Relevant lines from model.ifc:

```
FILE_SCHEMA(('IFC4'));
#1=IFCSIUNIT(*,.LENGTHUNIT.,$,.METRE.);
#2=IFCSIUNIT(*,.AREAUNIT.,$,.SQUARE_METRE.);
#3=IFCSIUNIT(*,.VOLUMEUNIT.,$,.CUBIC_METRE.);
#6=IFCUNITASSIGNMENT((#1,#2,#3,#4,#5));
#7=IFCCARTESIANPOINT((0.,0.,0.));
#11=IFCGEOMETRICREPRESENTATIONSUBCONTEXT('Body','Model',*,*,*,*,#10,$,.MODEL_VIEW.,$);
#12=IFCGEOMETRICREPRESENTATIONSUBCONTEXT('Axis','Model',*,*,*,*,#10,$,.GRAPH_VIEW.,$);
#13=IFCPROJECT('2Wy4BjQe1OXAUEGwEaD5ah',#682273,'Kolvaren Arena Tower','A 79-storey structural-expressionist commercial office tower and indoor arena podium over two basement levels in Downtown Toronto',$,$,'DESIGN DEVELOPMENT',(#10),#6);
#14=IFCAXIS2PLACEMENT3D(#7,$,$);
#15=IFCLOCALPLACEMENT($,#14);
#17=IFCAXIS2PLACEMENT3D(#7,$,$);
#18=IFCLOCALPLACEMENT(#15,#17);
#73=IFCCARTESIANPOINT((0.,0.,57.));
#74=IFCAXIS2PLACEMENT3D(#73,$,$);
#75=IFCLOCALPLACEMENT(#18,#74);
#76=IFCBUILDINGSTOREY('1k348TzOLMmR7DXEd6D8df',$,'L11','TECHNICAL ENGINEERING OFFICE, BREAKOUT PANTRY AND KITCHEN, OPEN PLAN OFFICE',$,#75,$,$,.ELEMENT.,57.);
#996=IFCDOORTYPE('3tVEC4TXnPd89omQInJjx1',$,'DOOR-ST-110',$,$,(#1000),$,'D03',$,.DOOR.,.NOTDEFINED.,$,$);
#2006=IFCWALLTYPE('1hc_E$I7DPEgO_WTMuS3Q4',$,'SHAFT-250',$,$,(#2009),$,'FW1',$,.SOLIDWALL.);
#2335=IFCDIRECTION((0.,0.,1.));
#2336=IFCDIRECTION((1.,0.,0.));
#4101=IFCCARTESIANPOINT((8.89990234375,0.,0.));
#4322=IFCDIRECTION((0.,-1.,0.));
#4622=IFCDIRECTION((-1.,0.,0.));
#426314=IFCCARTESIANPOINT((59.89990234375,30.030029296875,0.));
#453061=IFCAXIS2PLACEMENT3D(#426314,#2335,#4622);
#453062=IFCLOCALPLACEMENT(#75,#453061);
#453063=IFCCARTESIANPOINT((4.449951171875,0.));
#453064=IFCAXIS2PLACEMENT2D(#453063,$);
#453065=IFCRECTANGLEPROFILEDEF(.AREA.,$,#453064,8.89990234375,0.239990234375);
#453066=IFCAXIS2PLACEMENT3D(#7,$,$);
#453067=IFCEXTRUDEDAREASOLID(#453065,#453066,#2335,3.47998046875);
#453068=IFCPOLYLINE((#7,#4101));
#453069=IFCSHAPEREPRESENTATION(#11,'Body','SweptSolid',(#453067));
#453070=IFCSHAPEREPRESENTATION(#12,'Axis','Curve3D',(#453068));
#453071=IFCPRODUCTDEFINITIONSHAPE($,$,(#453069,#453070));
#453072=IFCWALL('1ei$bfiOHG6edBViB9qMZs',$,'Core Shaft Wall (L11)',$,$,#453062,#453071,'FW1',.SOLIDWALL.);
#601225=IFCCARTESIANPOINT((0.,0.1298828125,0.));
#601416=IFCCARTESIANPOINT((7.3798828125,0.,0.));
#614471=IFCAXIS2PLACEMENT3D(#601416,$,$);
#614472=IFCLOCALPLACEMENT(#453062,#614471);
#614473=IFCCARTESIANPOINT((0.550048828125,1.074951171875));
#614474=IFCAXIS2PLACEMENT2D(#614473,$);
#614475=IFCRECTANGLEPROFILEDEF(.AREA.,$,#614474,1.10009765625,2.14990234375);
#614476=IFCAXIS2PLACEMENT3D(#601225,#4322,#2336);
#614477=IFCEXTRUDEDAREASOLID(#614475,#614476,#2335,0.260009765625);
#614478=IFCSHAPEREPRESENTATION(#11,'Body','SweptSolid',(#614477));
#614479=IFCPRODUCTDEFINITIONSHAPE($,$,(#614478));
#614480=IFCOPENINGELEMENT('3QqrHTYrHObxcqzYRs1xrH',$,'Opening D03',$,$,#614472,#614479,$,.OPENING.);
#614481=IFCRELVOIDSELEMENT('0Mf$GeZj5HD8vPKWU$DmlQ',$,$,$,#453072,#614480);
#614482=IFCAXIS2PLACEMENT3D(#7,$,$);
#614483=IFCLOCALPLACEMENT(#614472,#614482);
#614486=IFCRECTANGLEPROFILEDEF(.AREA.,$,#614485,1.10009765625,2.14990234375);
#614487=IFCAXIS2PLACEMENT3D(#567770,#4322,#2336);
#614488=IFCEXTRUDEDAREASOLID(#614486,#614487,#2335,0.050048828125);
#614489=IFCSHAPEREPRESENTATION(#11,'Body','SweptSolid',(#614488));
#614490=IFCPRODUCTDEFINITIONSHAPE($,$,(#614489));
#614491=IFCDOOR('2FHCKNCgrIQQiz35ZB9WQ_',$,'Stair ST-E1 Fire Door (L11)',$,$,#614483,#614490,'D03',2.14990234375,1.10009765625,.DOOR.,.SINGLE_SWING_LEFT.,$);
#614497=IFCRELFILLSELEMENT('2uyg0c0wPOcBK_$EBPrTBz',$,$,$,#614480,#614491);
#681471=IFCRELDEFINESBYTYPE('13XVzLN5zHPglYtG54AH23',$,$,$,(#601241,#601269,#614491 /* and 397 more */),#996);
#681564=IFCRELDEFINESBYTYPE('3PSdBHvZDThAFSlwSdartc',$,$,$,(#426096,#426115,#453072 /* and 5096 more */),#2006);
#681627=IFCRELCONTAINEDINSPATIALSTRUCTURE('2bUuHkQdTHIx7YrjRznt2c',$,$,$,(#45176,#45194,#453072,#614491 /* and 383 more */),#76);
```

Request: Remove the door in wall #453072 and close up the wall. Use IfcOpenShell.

```python
import ifcopenshell
import ifcopenshell.api.feature
import ifcopenshell.api.root
import ifcopenshell.geom
import ifcopenshell.util.shape

model = ifcopenshell.open("model.ifc")
settings = ifcopenshell.geom.settings()


def volume(element):
    """Net volume in cubic metres, openings subtracted."""
    shape = ifcopenshell.geom.create_shape(settings, element)
    return ifcopenshell.util.shape.get_volume(shape.geometry)


door = model.by_guid("2FHCKNCgrIQQiz35ZB9WQ_")
opening = door.FillsVoids[0].RelatingOpeningElement
wall = opening.VoidsElements[0].RelatingBuildingElement
before = volume(wall)

ifcopenshell.api.root.remove_product(model, product=door)
ifcopenshell.api.feature.remove_feature(model, feature=opening)

after = volume(wall)

print(f"wall volume {before:.3f} -> {after:.3f} m3")

model.write("model-out.ifc")
```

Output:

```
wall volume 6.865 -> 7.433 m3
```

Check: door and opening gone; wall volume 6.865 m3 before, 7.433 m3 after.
